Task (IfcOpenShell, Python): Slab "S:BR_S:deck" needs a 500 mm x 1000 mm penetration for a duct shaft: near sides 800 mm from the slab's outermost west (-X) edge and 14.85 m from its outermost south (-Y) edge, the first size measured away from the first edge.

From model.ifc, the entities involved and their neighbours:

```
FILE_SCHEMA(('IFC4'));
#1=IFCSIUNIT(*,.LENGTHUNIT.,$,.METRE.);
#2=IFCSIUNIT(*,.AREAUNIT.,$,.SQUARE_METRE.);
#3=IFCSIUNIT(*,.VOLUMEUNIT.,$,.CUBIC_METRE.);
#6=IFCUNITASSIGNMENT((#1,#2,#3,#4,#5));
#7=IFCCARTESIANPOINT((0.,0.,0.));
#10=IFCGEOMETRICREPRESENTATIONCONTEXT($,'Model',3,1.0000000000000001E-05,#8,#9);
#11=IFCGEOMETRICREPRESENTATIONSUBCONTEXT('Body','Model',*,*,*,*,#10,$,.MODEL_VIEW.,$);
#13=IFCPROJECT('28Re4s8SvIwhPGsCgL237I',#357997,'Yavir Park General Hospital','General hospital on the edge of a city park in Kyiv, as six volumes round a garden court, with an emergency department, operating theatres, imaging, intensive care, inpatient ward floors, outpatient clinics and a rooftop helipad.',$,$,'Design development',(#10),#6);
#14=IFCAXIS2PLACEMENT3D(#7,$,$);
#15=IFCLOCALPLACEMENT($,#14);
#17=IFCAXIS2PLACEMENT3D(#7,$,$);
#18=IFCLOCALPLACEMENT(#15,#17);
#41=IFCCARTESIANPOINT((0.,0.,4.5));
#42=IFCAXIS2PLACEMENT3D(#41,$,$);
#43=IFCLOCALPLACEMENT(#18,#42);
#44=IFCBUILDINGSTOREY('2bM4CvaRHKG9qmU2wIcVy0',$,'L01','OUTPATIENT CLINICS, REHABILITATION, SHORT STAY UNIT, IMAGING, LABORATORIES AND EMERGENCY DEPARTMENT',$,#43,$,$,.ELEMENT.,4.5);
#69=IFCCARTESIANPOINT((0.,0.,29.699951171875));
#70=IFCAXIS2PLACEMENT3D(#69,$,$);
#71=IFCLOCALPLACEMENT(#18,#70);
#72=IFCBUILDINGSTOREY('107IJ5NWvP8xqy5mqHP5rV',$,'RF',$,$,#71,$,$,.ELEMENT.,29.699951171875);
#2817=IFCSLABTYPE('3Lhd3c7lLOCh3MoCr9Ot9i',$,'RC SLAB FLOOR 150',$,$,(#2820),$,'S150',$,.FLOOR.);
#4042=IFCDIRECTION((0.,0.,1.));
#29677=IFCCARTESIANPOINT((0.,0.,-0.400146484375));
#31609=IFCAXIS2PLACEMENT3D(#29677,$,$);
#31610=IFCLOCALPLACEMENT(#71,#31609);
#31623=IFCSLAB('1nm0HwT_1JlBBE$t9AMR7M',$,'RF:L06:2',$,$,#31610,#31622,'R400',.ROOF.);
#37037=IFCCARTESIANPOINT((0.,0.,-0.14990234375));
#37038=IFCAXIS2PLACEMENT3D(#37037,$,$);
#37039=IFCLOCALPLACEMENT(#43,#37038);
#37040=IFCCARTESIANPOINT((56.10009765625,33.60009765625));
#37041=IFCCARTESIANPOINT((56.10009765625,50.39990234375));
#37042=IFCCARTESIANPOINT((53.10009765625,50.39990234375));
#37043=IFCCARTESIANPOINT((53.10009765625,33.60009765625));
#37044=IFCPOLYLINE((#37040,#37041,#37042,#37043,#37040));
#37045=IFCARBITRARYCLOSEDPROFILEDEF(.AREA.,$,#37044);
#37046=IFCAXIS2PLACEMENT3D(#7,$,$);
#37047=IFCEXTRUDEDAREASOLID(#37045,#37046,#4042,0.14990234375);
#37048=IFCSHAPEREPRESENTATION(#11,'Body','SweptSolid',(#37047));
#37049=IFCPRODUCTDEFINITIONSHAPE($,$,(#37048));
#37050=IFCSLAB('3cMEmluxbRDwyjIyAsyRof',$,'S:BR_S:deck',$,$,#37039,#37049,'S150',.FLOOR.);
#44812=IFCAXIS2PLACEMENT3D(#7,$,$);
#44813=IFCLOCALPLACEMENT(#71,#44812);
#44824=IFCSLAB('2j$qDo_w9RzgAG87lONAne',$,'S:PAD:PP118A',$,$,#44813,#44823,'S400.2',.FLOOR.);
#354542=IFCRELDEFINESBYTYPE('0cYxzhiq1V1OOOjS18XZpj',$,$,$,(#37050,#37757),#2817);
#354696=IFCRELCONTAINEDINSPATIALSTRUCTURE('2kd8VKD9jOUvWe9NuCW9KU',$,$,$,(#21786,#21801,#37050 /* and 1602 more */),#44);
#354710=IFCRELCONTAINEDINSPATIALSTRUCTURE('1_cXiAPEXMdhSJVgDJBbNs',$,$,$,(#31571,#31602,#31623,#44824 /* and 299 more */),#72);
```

```python
import numpy as np
import ifcopenshell
import ifcopenshell.api.feature
import ifcopenshell.api.geometry
import ifcopenshell.api.root
import ifcopenshell.geom
import ifcopenshell.util.placement
import ifcopenshell.util.representation
import ifcopenshell.util.shape
import ifcopenshell.util.unit

model = ifcopenshell.open("model.ifc")
unit_scale = ifcopenshell.util.unit.calculate_unit_scale(model)
settings = ifcopenshell.geom.settings()


def volume(element):
    """Net volume in cubic metres, openings subtracted."""
    shape = ifcopenshell.geom.create_shape(settings, element)
    return ifcopenshell.util.shape.get_volume(shape.geometry)


slab = model.by_guid("3cMEmluxbRDwyjIyAsyRof")
before = volume(slab)

# Extent in the slab's own axes, in metres. The edges named are its -X and -Y sides.
slab_shape = ifcopenshell.geom.create_shape(settings, slab)
vertices = ifcopenshell.util.shape.get_vertices(slab_shape.geometry)
x_min, y_min, bottom = vertices.min(axis=0)
top = vertices[:, 2].max()

opening = ifcopenshell.api.root.create_entity(model, ifc_class="IfcOpeningElement", name="Duct shaft opening", predefined_type="OPENING")
context = ifcopenshell.util.representation.get_context(model, "Model", "Body", "MODEL_VIEW")
width, depth = 0.5, 1
outline = [(0.0, 0.0), (width, 0.0), (width, depth), (0.0, depth), (0.0, 0.0)]
# Overshoot both faces by 50 mm so the cut is clean.
shape = ifcopenshell.api.geometry.add_slab_representation(
    model, context=context, depth=top - bottom + 0.1, polyline=outline
)
ifcopenshell.api.geometry.assign_representation(model, product=opening, representation=shape)

matrix = ifcopenshell.util.placement.get_local_placement(slab.ObjectPlacement)
matrix[:, 3] = matrix @ np.append(np.array([x_min + 0.8, y_min + 14.85, bottom - 0.05]) / unit_scale, 1.0)
ifcopenshell.api.geometry.edit_object_placement(model, product=opening, matrix=matrix, is_si=False)
ifcopenshell.api.feature.add_feature(model, feature=opening, element=slab)

after = volume(slab)

print(f"slab volume {before:.3f} -> {after:.3f} m3")

model.write("model_rev.ifc")
```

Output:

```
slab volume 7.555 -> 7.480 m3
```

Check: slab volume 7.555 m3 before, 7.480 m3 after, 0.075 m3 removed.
